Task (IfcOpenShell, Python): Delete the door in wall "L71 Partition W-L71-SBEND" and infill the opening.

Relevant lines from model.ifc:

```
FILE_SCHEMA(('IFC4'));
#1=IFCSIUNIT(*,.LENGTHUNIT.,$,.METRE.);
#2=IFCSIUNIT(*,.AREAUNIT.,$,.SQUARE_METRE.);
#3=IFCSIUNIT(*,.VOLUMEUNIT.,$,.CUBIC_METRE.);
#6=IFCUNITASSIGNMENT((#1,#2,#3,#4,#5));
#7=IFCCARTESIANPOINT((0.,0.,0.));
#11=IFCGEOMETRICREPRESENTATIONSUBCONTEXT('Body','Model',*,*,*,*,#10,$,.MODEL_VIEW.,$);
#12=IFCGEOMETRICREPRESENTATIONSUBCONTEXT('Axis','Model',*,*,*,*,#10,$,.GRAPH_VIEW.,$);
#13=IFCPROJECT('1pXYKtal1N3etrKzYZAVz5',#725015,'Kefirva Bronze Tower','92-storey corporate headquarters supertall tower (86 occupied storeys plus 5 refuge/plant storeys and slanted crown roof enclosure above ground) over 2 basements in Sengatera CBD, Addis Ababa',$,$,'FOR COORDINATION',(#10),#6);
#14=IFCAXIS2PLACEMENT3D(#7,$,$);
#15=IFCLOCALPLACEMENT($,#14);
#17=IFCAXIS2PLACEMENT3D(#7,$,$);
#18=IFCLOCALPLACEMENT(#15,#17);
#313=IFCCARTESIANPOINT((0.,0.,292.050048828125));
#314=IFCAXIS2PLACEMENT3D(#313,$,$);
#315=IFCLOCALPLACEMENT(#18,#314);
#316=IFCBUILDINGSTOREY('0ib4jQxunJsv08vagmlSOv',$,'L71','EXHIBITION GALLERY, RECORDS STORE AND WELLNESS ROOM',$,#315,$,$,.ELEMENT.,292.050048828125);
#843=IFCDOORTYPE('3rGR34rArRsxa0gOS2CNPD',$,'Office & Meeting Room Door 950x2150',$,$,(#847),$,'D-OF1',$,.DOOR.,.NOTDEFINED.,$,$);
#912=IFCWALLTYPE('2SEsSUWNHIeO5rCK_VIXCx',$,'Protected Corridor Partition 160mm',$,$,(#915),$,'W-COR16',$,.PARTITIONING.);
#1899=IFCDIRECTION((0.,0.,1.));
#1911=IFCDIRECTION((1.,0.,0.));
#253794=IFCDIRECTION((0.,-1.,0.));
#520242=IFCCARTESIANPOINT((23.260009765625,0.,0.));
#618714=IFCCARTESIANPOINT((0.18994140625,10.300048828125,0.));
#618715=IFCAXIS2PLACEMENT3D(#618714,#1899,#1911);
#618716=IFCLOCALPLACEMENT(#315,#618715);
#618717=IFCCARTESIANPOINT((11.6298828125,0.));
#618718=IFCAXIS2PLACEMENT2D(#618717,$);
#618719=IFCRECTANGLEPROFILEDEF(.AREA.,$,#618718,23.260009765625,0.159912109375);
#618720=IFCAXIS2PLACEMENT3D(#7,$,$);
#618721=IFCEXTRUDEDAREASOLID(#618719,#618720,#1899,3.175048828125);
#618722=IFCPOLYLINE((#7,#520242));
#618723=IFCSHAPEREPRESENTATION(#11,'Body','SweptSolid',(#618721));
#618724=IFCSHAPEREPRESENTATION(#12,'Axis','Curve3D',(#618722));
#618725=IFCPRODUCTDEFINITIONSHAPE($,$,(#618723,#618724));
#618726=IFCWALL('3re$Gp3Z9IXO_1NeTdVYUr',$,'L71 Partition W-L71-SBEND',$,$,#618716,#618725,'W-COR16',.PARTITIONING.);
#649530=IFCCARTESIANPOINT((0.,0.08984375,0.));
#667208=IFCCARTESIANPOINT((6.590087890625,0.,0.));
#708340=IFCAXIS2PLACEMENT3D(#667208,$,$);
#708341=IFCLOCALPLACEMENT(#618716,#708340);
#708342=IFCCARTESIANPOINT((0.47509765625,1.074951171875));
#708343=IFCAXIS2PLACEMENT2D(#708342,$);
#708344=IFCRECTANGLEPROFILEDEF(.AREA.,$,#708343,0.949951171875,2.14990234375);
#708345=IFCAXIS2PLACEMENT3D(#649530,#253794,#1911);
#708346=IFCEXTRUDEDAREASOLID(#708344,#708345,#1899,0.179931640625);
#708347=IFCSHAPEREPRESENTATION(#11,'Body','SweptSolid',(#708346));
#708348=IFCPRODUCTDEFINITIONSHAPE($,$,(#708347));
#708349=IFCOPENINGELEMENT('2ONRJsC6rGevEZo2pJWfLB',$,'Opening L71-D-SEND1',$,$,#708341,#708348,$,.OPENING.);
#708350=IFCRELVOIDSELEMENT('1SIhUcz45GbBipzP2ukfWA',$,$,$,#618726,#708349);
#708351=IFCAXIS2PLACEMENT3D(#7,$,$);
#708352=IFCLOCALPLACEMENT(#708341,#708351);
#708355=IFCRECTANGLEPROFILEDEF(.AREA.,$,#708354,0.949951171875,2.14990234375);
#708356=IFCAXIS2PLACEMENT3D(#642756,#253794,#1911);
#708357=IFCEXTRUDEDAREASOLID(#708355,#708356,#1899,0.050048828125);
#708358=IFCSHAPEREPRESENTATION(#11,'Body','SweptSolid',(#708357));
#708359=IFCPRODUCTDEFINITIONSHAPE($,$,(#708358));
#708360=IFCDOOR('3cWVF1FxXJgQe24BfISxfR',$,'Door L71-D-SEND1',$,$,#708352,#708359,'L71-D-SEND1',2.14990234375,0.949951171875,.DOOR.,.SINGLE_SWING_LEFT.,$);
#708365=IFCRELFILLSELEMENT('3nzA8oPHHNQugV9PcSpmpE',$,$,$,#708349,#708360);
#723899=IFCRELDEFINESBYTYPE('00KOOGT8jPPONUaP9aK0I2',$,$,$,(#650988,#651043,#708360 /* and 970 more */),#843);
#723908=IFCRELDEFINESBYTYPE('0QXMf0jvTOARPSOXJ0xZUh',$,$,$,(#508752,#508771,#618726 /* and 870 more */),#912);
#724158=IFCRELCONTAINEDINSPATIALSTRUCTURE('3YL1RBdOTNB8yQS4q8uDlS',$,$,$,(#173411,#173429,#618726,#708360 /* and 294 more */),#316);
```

```python
import ifcopenshell
import ifcopenshell.api.feature
import ifcopenshell.api.root
import ifcopenshell.geom
import ifcopenshell.util.shape

model = ifcopenshell.open("model.ifc")
settings = ifcopenshell.geom.settings()


def volume(element):
    """Net volume in cubic metres, openings subtracted."""
    shape = ifcopenshell.geom.create_shape(settings, element)
    return ifcopenshell.util.shape.get_volume(shape.geometry)


door = model.by_id(708360)
opening = door.FillsVoids[0].RelatingOpeningElement
wall = opening.VoidsElements[0].RelatingBuildingElement
before = volume(wall)

ifcopenshell.api.root.remove_product(model, product=door)
ifcopenshell.api.feature.remove_feature(model, feature=opening)

after = volume(wall)

print(f"wall volume {before:.3f} -> {after:.3f} m3")

model.write("model_v2.ifc")
```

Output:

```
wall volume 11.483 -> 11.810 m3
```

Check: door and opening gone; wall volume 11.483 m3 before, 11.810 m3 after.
